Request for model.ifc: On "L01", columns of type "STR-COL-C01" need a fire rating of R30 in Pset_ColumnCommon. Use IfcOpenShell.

First a look at what the model holds.

```python
import ifcopenshell
import ifcopenshell.util.element

model = ifcopenshell.open("model.ifc")
print(model.schema)
storey = next(s for s in model.by_type("IfcBuildingStorey") if s.Name == "L01")
columns = [e for e in ifcopenshell.util.element.get_decomposition(storey) if e.is_a("IfcColumn")]
seen = {}
for e in columns:
    element_type = ifcopenshell.util.element.get_type(e)
    key = (element_type.Name if element_type != e and element_type else None, ifcopenshell.util.element.get_pset(e, "Pset_ColumnCommon", "FireRating"))
    seen[key] = seen.get(key, 0) + 1
for (name, value), count in sorted(seen.items(), key=str):
    print(count, "x", name, "|", value)
```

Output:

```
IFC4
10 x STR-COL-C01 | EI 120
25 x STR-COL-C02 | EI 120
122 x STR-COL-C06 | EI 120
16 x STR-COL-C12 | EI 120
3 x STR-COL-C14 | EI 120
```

```python
import ifcopenshell
import ifcopenshell.api.pset
import ifcopenshell.util.element

model = ifcopenshell.open("model.ifc")

storey = next(s for s in model.by_type("IfcBuildingStorey") if s.Name == "L01")
columns = [e for e in ifcopenshell.util.element.get_decomposition(storey) if e.is_a("IfcColumn")]

count = 0
for e in columns:
    element_type = ifcopenshell.util.element.get_type(e)
    if element_type in (None, e) or element_type.Name != "STR-COL-C01":
        continue
    # add_pset returns the element's existing set when there is one.
    pset = ifcopenshell.api.pset.add_pset(model, product=e, name="Pset_ColumnCommon")
    ifcopenshell.api.pset.edit_pset(model, pset=pset, properties={"FireRating": "R30"})
    count += 1

print(count, "columns updated")

model.write("model-out.ifc")
```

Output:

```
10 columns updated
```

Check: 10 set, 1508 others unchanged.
